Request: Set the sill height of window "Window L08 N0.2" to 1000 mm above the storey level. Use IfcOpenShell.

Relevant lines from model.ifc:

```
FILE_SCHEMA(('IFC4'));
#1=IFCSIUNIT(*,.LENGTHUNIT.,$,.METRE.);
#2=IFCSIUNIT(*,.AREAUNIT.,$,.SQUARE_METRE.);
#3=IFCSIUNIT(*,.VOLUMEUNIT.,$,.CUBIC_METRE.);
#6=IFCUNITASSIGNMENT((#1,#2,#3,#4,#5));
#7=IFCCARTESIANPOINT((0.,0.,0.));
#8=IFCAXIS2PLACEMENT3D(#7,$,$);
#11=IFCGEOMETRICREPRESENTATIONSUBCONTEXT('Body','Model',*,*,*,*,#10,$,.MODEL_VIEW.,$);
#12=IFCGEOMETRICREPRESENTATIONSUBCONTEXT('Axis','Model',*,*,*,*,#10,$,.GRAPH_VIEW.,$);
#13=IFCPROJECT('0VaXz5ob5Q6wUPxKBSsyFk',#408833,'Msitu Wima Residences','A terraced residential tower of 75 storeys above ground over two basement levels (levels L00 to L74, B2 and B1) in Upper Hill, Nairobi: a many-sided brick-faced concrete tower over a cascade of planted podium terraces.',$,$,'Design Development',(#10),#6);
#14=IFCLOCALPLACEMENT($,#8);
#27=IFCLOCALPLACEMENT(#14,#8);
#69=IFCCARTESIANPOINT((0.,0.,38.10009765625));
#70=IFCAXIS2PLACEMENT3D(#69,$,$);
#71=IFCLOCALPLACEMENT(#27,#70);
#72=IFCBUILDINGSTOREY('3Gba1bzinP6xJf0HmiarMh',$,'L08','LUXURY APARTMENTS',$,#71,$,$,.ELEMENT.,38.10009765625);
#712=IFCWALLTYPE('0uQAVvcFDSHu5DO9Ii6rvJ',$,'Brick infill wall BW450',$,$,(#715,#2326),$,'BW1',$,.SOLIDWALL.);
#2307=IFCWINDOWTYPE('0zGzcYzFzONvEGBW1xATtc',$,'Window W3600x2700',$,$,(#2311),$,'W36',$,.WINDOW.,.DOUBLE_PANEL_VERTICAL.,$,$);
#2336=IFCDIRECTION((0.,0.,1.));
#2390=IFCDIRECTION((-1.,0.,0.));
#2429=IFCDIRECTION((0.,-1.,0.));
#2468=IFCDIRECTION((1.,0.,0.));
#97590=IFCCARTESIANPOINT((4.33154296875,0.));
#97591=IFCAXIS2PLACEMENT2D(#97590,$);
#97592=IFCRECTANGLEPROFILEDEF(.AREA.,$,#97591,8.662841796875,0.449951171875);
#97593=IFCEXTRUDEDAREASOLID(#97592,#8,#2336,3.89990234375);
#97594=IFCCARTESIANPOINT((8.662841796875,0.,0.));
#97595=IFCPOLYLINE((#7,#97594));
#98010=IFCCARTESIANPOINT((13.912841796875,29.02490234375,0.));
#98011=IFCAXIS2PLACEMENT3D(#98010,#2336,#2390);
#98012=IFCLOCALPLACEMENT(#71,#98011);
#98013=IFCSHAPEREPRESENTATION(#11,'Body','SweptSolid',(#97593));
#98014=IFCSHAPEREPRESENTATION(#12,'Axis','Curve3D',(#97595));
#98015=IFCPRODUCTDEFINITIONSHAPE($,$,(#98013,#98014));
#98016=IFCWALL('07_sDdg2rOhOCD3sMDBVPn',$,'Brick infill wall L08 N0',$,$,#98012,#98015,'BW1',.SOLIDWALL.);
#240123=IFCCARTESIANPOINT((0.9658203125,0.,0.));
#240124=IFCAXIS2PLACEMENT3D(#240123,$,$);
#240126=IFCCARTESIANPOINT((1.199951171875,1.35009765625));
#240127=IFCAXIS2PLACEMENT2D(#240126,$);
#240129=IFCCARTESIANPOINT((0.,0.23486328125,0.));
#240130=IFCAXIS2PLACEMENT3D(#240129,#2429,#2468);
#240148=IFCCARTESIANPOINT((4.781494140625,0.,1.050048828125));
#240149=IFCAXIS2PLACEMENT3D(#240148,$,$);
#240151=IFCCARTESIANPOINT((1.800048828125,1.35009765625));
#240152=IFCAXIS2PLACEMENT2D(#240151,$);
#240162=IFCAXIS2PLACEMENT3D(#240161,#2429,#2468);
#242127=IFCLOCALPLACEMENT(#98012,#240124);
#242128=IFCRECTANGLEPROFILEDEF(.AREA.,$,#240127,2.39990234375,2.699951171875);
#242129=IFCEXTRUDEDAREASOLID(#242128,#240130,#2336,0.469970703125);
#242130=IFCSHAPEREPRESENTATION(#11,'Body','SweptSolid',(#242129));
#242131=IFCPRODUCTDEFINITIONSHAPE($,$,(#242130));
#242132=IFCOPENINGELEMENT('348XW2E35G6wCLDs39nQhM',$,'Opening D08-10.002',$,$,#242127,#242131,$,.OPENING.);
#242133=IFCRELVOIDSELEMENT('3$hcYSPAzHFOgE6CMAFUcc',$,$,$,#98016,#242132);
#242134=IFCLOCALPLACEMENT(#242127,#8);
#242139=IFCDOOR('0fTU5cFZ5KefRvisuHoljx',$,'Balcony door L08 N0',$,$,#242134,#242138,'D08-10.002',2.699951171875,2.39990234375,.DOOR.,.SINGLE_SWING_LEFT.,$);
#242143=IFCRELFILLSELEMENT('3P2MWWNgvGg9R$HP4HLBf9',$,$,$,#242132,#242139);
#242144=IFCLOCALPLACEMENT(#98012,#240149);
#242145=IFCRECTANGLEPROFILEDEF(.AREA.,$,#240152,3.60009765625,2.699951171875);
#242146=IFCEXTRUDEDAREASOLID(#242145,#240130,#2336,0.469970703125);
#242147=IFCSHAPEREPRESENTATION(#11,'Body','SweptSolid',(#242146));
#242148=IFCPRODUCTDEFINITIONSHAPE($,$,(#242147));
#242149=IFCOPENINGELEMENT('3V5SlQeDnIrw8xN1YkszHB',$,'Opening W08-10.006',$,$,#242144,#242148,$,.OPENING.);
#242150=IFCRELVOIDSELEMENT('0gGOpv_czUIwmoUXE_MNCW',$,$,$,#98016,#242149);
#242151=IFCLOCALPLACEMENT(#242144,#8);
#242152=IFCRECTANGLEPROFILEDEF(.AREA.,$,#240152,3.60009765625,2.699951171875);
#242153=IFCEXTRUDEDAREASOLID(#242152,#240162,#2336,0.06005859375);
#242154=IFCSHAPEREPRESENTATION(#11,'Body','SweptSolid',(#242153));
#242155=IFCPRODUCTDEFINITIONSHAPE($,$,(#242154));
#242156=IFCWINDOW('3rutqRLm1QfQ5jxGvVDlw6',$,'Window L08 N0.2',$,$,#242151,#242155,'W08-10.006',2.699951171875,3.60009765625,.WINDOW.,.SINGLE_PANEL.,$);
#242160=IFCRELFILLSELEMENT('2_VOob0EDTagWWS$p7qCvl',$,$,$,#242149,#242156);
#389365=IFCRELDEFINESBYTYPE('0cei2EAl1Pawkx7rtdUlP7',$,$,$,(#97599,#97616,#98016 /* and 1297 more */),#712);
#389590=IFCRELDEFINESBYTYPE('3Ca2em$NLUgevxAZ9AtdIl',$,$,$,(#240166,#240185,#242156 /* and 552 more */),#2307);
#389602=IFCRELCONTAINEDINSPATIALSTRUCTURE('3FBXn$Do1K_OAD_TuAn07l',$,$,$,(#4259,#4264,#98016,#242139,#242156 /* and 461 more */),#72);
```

```python
import numpy as np
import ifcopenshell
import ifcopenshell.api.geometry
import ifcopenshell.geom
import ifcopenshell.util.element
import ifcopenshell.util.placement
import ifcopenshell.util.shape
import ifcopenshell.util.unit

model = ifcopenshell.open("model.ifc")
unit_scale = ifcopenshell.util.unit.calculate_unit_scale(model)

window = model.by_guid("3rutqRLm1QfQ5jxGvVDlw6")
opening = window.FillsVoids[0].RelatingOpeningElement
storey = ifcopenshell.util.element.get_container(window, ifc_class="IfcBuildingStorey")
level = ifcopenshell.util.placement.get_local_placement(storey.ObjectPlacement)[2, 3]

# The opening's origin need not be at the sill, so measure its lowest point.
shape = ifcopenshell.geom.create_shape(ifcopenshell.geom.settings(), opening)
bottom = ifcopenshell.util.shape.get_shape_bottom_elevation(shape, shape.geometry) / unit_scale
dz = level + 1.0 - bottom

shift = np.array([0.0, 0.0, dz])
# The window is placed relative to its opening, so it follows when the opening moves.
matrix = ifcopenshell.util.placement.get_local_placement(opening.ObjectPlacement)
matrix[:3, 3] += shift
ifcopenshell.api.geometry.edit_object_placement(
    model, product=opening, matrix=matrix, is_si=False, should_transform_children=True
)

print(f"moved by {dz * unit_scale:+.3f} m")

model.write("model_rev.ifc")
```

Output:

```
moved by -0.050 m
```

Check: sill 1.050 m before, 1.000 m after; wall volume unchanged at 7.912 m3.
